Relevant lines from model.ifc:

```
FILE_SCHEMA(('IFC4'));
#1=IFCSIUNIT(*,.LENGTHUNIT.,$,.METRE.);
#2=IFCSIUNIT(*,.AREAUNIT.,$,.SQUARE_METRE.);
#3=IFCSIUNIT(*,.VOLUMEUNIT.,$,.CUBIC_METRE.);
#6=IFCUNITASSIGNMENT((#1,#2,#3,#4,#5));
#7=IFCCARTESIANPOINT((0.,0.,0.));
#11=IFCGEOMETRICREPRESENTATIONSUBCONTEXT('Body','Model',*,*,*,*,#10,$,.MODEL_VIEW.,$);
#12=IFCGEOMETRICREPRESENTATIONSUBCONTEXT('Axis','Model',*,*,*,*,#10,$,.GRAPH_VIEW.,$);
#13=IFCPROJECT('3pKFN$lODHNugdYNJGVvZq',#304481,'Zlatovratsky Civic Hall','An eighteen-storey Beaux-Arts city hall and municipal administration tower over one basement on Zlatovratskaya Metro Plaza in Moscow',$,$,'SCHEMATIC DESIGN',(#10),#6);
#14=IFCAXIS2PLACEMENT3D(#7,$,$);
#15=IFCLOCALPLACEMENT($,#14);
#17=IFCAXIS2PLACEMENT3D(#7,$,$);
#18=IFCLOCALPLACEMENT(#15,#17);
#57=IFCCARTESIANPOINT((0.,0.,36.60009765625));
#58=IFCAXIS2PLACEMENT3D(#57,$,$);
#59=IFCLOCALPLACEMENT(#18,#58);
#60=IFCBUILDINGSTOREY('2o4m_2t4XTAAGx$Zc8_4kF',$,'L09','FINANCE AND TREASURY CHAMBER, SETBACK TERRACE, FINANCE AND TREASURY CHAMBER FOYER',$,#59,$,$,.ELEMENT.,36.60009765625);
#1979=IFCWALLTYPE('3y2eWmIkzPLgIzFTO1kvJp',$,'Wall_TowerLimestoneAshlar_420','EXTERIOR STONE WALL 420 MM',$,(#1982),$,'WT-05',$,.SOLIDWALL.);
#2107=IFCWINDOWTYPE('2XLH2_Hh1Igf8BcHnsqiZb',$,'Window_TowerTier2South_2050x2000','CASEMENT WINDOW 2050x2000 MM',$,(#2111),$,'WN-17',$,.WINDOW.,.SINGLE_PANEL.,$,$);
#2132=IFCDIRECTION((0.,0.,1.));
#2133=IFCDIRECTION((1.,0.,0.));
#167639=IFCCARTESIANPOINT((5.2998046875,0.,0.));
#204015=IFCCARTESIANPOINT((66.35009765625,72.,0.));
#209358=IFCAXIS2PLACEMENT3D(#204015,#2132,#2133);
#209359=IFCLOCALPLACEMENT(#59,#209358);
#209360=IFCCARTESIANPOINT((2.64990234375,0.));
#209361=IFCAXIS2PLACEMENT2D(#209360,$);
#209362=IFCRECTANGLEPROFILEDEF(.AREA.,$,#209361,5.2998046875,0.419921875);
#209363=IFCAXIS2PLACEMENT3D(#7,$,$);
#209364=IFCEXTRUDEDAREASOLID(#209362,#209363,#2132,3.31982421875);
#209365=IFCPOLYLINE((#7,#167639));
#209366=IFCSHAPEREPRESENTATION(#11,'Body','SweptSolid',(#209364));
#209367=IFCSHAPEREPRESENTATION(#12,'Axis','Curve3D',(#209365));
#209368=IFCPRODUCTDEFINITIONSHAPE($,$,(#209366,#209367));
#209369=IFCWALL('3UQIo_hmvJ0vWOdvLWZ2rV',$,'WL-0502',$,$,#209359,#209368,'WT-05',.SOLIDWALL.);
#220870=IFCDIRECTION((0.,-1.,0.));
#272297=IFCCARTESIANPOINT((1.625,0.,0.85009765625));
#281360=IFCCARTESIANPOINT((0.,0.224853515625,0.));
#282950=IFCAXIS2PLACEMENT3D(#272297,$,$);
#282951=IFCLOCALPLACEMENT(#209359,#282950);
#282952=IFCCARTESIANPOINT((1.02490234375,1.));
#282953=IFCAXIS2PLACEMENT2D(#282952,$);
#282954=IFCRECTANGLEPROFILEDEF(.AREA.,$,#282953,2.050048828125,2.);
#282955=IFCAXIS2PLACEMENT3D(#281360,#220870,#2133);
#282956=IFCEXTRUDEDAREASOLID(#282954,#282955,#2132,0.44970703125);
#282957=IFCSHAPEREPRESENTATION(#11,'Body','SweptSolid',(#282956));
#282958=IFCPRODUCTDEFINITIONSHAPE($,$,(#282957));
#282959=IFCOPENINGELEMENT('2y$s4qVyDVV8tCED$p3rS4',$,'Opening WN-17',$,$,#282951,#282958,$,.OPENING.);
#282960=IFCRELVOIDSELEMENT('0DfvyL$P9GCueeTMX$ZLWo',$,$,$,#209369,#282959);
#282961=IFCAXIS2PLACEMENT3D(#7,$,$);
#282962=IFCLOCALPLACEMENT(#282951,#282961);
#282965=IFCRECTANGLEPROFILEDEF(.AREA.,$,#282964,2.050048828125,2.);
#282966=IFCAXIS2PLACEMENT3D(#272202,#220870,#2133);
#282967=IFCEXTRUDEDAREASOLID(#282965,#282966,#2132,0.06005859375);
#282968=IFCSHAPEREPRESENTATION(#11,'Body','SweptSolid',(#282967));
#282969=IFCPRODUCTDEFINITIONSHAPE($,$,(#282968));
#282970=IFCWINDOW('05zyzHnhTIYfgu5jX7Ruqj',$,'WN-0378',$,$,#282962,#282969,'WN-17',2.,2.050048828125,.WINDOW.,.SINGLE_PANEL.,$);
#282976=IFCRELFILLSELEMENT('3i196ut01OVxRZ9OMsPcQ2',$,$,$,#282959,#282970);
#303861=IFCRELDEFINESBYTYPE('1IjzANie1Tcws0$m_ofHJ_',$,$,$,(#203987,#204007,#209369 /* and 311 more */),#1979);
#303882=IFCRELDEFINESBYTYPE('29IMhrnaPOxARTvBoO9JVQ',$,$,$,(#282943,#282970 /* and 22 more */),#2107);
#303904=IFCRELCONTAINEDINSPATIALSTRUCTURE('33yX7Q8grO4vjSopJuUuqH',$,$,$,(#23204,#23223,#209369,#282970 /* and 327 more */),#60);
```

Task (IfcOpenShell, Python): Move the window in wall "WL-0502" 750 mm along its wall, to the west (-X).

```python
import ifcopenshell
import ifcopenshell.api.geometry
import ifcopenshell.util.placement
import ifcopenshell.util.unit

model = ifcopenshell.open("model.ifc")
unit_scale = ifcopenshell.util.unit.calculate_unit_scale(model)

window = model.by_id(282970)
opening = window.FillsVoids[0].RelatingOpeningElement
wall = opening.VoidsElements[0].RelatingBuildingElement

wall_matrix = ifcopenshell.util.placement.get_local_placement(wall.ObjectPlacement)
shift = wall_matrix[:3, 0] * -0.75 / unit_scale
before = ifcopenshell.util.placement.get_local_placement(window.ObjectPlacement)[:3, 3].copy()

# The window is placed relative to its opening, so it follows when the opening moves.
matrix = ifcopenshell.util.placement.get_local_placement(opening.ObjectPlacement)
matrix[:3, 3] += shift
ifcopenshell.api.geometry.edit_object_placement(
    model, product=opening, matrix=matrix, is_si=False, should_transform_children=True
)

after = ifcopenshell.util.placement.get_local_placement(window.ObjectPlacement)[:3, 3]
print("window moved by", (after - before).round(3) + 0.0)

model.write("model_updated.ifc")
```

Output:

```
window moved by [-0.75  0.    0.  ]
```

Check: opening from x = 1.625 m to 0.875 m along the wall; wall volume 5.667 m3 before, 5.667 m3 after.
